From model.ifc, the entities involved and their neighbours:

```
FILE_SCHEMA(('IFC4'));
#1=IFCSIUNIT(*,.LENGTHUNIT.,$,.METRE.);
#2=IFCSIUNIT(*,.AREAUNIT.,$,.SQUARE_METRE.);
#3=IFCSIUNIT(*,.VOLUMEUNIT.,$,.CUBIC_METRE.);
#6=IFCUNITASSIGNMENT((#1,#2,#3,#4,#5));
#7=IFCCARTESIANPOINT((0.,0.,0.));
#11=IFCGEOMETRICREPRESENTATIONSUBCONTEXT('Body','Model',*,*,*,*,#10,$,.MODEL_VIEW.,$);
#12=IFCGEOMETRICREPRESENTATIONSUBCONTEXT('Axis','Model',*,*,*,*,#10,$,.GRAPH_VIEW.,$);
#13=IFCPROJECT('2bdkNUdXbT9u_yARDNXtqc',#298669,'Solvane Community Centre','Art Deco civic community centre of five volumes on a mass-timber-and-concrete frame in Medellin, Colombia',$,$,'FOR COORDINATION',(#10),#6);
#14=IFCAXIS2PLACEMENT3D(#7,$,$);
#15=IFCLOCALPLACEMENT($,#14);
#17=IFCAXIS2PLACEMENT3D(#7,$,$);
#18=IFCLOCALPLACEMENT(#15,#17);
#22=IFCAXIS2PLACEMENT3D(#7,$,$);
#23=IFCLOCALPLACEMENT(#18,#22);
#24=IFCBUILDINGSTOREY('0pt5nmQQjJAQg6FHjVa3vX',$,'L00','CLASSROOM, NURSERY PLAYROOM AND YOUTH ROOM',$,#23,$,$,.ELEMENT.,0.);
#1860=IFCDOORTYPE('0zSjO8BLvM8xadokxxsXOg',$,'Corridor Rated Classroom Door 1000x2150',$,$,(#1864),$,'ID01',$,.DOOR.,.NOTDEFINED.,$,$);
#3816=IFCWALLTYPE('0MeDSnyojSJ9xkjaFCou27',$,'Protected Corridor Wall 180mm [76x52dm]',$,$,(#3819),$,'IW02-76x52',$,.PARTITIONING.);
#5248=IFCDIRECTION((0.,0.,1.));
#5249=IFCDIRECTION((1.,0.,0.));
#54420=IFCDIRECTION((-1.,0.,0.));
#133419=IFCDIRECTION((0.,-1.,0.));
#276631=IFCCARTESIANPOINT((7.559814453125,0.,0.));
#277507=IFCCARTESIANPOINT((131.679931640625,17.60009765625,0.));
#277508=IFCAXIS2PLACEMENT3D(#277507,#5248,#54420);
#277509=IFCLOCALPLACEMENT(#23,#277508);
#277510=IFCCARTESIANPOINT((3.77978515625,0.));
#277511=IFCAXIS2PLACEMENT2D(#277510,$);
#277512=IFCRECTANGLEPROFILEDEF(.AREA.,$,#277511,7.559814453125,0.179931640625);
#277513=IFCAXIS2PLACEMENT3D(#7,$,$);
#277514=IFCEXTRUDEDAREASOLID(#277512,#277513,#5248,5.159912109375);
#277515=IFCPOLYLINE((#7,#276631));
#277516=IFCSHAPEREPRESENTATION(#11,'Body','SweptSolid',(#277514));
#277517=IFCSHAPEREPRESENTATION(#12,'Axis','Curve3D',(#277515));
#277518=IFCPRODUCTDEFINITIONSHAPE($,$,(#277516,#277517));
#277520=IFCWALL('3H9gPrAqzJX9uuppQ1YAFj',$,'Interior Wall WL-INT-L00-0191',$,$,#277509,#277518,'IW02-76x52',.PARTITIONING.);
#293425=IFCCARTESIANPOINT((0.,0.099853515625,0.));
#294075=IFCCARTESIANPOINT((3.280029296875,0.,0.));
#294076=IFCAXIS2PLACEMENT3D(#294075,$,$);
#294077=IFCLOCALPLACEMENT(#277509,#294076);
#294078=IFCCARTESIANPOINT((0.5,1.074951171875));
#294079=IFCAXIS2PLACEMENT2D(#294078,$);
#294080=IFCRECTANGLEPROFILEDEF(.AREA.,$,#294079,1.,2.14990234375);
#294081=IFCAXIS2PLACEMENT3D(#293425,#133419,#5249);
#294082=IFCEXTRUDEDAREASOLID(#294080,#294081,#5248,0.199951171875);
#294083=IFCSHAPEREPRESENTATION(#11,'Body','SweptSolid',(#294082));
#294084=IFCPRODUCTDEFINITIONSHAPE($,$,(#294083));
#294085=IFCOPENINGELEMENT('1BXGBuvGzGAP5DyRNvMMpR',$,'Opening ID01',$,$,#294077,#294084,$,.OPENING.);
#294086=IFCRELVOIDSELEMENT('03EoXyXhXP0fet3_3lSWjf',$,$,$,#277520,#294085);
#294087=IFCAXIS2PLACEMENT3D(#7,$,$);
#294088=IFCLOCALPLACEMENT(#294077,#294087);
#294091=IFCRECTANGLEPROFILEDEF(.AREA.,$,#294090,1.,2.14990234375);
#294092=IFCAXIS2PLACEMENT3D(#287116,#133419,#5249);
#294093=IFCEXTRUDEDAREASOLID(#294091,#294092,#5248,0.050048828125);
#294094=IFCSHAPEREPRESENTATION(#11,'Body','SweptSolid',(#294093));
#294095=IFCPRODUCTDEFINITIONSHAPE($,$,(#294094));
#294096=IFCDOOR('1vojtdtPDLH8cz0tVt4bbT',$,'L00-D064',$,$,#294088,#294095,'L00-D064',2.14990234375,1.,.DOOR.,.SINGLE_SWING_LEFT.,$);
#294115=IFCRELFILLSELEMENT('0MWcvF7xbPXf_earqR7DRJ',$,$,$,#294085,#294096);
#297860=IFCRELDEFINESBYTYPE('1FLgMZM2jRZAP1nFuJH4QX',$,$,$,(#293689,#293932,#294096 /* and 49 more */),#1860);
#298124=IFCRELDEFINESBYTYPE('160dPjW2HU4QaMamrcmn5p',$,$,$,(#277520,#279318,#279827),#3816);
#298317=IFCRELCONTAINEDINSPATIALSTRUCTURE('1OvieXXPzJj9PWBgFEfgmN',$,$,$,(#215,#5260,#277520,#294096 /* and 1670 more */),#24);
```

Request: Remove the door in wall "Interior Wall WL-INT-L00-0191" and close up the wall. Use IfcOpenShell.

```python
import ifcopenshell
import ifcopenshell.api.feature
import ifcopenshell.api.root
import ifcopenshell.geom
import ifcopenshell.util.shape

model = ifcopenshell.open("model.ifc")
settings = ifcopenshell.geom.settings()


def volume(element):
    """Net volume in cubic metres, openings subtracted."""
    shape = ifcopenshell.geom.create_shape(settings, element)
    return ifcopenshell.util.shape.get_volume(shape.geometry)


door = model.by_id(294096)
opening = door.FillsVoids[0].RelatingOpeningElement
wall = opening.VoidsElements[0].RelatingBuildingElement
before = volume(wall)

ifcopenshell.api.root.remove_product(model, product=door)
ifcopenshell.api.feature.remove_feature(model, feature=opening)

after = volume(wall)

print(f"wall volume {before:.3f} -> {after:.3f} m3")

model.write("model_edited.ifc")
```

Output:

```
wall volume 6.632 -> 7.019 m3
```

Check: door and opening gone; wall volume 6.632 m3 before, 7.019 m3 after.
